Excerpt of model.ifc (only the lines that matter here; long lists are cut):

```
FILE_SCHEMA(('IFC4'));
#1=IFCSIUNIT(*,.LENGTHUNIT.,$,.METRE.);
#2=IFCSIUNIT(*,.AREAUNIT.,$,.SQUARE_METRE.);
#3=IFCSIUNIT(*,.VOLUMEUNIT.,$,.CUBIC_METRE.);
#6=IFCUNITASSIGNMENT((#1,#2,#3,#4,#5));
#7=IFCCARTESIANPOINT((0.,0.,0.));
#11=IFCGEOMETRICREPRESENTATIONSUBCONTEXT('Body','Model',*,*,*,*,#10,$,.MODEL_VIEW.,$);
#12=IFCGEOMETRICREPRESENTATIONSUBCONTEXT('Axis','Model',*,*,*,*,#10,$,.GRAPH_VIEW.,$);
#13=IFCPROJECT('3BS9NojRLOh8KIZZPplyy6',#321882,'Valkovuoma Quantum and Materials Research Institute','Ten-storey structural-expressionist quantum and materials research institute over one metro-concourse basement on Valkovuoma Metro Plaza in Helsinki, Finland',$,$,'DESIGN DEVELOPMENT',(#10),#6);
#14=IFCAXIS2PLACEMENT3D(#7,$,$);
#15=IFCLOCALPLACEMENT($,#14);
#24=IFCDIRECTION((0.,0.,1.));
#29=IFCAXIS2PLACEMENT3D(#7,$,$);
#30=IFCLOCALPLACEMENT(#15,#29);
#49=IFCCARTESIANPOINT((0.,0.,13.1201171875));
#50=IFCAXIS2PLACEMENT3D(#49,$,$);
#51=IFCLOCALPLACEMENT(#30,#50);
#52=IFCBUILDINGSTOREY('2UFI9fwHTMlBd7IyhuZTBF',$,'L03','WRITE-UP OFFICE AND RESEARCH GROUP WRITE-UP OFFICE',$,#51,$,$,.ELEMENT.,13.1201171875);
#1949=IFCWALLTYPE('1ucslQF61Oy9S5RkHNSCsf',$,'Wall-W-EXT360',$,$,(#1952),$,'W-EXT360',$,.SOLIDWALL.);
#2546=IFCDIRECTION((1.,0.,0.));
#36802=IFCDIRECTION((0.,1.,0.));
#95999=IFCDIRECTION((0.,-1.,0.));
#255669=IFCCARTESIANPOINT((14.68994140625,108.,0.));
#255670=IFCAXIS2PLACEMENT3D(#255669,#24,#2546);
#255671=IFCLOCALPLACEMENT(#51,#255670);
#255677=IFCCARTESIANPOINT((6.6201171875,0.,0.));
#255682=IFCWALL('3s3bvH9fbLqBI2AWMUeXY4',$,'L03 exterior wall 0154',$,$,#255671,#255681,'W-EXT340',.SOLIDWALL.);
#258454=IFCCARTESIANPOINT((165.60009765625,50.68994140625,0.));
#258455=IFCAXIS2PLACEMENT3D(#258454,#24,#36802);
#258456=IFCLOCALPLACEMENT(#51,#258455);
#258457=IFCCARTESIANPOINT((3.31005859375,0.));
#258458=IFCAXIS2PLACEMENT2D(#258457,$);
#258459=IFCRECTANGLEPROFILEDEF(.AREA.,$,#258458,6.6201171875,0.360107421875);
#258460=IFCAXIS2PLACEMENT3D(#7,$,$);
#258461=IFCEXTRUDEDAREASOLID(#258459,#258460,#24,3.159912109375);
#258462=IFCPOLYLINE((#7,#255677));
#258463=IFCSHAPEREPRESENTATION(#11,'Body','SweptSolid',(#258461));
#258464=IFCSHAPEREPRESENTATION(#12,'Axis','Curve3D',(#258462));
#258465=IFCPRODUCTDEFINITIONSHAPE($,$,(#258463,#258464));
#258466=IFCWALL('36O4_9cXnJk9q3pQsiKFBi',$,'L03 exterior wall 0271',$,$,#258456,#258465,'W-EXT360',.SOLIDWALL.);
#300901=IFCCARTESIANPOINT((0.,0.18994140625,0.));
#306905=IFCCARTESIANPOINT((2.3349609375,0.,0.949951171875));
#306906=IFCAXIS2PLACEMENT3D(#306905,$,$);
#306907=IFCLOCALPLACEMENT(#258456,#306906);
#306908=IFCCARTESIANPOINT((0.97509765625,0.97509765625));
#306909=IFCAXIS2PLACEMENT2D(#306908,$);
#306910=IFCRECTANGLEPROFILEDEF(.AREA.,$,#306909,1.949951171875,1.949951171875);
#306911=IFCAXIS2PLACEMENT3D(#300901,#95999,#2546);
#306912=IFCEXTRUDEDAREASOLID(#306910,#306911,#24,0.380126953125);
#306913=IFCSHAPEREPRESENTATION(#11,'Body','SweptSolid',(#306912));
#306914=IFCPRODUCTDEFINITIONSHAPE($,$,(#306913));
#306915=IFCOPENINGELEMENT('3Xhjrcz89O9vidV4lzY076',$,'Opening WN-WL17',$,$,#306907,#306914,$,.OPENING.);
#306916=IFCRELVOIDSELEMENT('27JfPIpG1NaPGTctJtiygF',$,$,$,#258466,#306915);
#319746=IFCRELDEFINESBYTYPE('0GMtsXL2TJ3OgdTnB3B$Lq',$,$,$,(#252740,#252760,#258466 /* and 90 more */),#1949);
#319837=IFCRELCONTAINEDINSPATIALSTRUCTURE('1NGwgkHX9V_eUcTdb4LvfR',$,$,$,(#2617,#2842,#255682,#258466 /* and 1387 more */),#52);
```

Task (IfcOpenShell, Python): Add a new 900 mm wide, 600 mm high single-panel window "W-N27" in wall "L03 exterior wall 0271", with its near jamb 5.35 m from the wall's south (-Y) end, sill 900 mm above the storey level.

```python
import numpy as np
import ifcopenshell
import ifcopenshell.api.feature
import ifcopenshell.api.geometry
import ifcopenshell.api.root
import ifcopenshell.api.spatial
import ifcopenshell.geom
import ifcopenshell.util.element
import ifcopenshell.util.placement
import ifcopenshell.util.representation
import ifcopenshell.util.shape
import ifcopenshell.util.unit

model = ifcopenshell.open("model.ifc")
unit_scale = ifcopenshell.util.unit.calculate_unit_scale(model)
settings = ifcopenshell.geom.settings()


def volume(element):
    """Net volume in cubic metres, openings subtracted."""
    shape = ifcopenshell.geom.create_shape(settings, element)
    return ifcopenshell.util.shape.get_volume(shape.geometry)


wall = model.by_id(258466)
storey = ifcopenshell.util.element.get_container(wall, ifc_class="IfcBuildingStorey")
context = ifcopenshell.util.representation.get_context(model, "Model", "Body", "MODEL_VIEW")
before = volume(wall)

width, height, from_end, sill = 0.9, 0.6, 5.35, 0.9  # metres

# The wall runs along its own X axis, and the end named is its -X end.
wall_shape = ifcopenshell.geom.create_shape(settings, wall)
x, y, z = ifcopenshell.util.shape.get_vertices(wall_shape.geometry).T
start = x.min() + from_end
face, thickness = float(y.min()), float(y.max() - y.min())
wall_matrix = ifcopenshell.util.placement.get_local_placement(wall.ObjectPlacement)
level = ifcopenshell.util.placement.get_local_placement(storey.ObjectPlacement)[2, 3]


def in_wall(x, y):
    """Placement at x, y metres in the wall's axes, at sill height."""
    matrix = wall_matrix.copy()
    matrix[:, 3] = wall_matrix @ np.array([x / unit_scale, y / unit_scale, 0.0, 1.0])
    matrix[2, 3] = level + sill / unit_scale
    return matrix


# Opening: a box that overshoots both wall faces by 50 mm.
opening = ifcopenshell.api.root.create_entity(model, ifc_class="IfcOpeningElement", predefined_type="OPENING")
box = ifcopenshell.api.geometry.add_wall_representation(
    model, context=context, length=width, height=height, thickness=thickness + 0.1
)
ifcopenshell.api.geometry.assign_representation(model, product=opening, representation=box)
ifcopenshell.api.geometry.edit_object_placement(model, product=opening, matrix=in_wall(start, face - 0.05), is_si=False)
ifcopenshell.api.feature.add_feature(model, feature=opening, element=wall)

window = ifcopenshell.api.root.create_entity(model, ifc_class="IfcWindow", name="W-N27", predefined_type="WINDOW")
window.OverallWidth, window.OverallHeight = width / unit_scale, height / unit_scale
window.PartitioningType = "SINGLE_PANEL"
body = ifcopenshell.api.geometry.add_window_representation(
    model,
    context=context,
    overall_width=window.OverallWidth,
    overall_height=window.OverallHeight,
    partition_type="SINGLE_PANEL",
)
ifcopenshell.api.geometry.assign_representation(model, product=window, representation=body)
ifcopenshell.api.spatial.assign_container(model, products=[window], relating_structure=storey)
ifcopenshell.api.feature.add_filling(model, opening=opening, element=window)

# Centre the window in the wall's thickness.
ifcopenshell.api.geometry.edit_object_placement(model, product=window, matrix=in_wall(start, face), is_si=False)
window_shape = ifcopenshell.geom.create_shape(settings, window)
depth = ifcopenshell.util.shape.get_vertices(window_shape.geometry)[:, 1]
offset = face + thickness / 2 - (depth.min() + depth.max()) / 2
ifcopenshell.api.geometry.edit_object_placement(model, product=window, matrix=in_wall(start, offset), is_si=False)

after = volume(wall)

print(f"wall volume {before:.3f} -> {after:.3f} m3")

model.write("model_updated.ifc")
```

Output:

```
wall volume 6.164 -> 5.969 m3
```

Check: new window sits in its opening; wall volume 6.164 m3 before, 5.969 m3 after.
